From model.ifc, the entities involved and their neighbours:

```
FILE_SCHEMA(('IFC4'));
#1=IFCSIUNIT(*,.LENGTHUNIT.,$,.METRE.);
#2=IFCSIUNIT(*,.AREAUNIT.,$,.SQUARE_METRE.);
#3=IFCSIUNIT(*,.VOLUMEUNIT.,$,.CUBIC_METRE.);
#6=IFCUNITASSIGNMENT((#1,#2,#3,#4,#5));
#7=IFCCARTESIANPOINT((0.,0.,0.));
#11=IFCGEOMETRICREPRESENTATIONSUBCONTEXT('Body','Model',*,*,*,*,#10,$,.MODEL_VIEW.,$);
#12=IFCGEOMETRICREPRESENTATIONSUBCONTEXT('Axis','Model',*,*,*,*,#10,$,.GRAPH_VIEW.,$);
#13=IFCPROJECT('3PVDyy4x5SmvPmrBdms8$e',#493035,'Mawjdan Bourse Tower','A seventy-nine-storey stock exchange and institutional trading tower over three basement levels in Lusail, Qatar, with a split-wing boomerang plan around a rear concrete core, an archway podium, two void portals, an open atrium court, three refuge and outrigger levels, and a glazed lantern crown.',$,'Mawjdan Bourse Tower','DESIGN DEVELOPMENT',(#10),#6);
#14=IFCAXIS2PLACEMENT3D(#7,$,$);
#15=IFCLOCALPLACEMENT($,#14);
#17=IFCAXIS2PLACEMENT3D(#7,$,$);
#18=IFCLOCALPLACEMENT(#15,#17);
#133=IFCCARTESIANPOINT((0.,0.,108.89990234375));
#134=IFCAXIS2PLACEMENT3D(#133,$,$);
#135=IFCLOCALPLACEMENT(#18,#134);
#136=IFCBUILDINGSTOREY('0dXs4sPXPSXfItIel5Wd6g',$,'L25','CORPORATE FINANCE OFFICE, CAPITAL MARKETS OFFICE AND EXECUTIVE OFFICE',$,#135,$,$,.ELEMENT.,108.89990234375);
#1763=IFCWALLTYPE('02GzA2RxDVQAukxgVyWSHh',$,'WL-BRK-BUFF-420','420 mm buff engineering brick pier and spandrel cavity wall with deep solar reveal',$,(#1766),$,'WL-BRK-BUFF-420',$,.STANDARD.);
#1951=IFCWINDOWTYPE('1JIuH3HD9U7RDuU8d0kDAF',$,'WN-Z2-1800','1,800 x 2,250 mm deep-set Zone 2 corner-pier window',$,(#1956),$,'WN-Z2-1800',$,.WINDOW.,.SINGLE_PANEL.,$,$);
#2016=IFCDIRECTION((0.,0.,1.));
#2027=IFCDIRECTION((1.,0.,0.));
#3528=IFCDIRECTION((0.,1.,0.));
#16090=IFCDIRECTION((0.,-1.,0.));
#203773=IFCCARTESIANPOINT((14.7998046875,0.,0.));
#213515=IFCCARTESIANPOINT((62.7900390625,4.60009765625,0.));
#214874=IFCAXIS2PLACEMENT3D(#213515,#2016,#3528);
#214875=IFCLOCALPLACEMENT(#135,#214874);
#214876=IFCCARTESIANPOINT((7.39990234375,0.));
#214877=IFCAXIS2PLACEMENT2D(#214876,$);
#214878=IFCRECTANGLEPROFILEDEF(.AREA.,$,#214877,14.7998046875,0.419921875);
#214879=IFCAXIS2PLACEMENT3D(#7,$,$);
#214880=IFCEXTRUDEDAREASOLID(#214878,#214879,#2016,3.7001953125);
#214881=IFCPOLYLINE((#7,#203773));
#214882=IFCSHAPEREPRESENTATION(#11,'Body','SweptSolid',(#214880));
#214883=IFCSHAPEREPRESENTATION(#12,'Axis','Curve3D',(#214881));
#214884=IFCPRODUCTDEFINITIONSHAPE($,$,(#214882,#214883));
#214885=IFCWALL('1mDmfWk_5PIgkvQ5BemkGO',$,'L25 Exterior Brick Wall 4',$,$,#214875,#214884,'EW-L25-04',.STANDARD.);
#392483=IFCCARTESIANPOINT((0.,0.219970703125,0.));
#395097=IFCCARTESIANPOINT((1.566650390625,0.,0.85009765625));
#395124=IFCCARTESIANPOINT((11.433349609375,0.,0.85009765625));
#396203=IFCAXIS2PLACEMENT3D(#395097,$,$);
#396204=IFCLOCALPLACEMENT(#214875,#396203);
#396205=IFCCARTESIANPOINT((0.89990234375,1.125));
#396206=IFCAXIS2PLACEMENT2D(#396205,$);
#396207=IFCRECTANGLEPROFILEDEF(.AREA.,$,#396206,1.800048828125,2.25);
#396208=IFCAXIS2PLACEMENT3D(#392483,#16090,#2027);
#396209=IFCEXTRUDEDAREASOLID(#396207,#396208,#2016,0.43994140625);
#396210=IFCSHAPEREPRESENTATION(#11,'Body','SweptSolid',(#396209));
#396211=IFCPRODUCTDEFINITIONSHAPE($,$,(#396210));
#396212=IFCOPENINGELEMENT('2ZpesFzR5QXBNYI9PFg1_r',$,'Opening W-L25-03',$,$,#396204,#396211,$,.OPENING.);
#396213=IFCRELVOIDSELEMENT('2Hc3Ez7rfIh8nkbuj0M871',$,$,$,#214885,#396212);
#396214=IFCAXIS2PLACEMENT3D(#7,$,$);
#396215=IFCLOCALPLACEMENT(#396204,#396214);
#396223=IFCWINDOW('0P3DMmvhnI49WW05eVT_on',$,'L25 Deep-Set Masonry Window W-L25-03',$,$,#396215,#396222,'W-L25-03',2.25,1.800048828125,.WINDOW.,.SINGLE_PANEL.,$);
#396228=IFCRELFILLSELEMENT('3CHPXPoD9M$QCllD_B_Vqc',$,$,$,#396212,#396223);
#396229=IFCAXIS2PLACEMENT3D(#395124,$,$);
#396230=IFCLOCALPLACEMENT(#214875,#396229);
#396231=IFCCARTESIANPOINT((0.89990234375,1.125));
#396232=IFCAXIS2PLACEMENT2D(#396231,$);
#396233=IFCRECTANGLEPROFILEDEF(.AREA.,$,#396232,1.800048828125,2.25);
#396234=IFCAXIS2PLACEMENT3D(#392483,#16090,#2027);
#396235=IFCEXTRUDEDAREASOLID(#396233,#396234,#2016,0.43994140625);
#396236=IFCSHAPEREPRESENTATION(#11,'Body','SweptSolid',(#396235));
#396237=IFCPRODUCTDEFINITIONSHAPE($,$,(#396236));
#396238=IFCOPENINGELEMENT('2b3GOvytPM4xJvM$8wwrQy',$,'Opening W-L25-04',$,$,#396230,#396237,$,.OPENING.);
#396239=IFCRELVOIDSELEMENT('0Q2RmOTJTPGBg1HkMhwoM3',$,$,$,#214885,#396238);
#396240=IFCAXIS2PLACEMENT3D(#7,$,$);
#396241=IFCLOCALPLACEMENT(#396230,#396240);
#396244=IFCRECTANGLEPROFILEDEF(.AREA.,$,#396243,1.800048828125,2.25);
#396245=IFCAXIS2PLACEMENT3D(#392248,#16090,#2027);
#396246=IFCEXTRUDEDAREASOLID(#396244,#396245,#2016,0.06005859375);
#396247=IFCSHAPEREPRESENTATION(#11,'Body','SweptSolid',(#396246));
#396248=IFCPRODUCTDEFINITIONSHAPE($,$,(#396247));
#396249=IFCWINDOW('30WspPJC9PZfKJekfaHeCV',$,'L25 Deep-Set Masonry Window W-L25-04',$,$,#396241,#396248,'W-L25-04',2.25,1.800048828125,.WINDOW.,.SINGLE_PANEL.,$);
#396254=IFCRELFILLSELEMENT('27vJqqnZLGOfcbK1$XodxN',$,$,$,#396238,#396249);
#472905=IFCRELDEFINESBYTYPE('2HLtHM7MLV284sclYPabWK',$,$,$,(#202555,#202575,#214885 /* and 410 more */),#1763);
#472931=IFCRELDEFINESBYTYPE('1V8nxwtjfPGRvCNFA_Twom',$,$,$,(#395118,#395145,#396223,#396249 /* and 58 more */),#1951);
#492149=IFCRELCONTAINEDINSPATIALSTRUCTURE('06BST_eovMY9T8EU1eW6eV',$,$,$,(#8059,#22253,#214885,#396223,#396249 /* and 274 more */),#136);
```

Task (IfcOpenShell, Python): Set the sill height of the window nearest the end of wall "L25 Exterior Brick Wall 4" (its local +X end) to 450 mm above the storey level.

```python
import numpy as np
import ifcopenshell
import ifcopenshell.api.geometry
import ifcopenshell.geom
import ifcopenshell.util.element
import ifcopenshell.util.placement
import ifcopenshell.util.shape
import ifcopenshell.util.unit

model = ifcopenshell.open("model.ifc")
unit_scale = ifcopenshell.util.unit.calculate_unit_scale(model)

window = model.by_guid("30WspPJC9PZfKJekfaHeCV")
opening = window.FillsVoids[0].RelatingOpeningElement
storey = ifcopenshell.util.element.get_container(window, ifc_class="IfcBuildingStorey")
level = ifcopenshell.util.placement.get_local_placement(storey.ObjectPlacement)[2, 3]

# The opening's origin need not be at the sill, so measure its lowest point.
shape = ifcopenshell.geom.create_shape(ifcopenshell.geom.settings(), opening)
bottom = ifcopenshell.util.shape.get_shape_bottom_elevation(shape, shape.geometry) / unit_scale
dz = level + 0.45 - bottom

shift = np.array([0.0, 0.0, dz])
# The window is placed relative to its opening, so it follows when the opening moves.
matrix = ifcopenshell.util.placement.get_local_placement(opening.ObjectPlacement)
matrix[:3, 3] += shift
ifcopenshell.api.geometry.edit_object_placement(
    model, product=opening, matrix=matrix, is_si=False, should_transform_children=True
)

print(f"moved by {dz * unit_scale:+.3f} m")

model.write("model_rev.ifc")
```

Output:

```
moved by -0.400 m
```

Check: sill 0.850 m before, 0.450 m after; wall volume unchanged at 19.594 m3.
